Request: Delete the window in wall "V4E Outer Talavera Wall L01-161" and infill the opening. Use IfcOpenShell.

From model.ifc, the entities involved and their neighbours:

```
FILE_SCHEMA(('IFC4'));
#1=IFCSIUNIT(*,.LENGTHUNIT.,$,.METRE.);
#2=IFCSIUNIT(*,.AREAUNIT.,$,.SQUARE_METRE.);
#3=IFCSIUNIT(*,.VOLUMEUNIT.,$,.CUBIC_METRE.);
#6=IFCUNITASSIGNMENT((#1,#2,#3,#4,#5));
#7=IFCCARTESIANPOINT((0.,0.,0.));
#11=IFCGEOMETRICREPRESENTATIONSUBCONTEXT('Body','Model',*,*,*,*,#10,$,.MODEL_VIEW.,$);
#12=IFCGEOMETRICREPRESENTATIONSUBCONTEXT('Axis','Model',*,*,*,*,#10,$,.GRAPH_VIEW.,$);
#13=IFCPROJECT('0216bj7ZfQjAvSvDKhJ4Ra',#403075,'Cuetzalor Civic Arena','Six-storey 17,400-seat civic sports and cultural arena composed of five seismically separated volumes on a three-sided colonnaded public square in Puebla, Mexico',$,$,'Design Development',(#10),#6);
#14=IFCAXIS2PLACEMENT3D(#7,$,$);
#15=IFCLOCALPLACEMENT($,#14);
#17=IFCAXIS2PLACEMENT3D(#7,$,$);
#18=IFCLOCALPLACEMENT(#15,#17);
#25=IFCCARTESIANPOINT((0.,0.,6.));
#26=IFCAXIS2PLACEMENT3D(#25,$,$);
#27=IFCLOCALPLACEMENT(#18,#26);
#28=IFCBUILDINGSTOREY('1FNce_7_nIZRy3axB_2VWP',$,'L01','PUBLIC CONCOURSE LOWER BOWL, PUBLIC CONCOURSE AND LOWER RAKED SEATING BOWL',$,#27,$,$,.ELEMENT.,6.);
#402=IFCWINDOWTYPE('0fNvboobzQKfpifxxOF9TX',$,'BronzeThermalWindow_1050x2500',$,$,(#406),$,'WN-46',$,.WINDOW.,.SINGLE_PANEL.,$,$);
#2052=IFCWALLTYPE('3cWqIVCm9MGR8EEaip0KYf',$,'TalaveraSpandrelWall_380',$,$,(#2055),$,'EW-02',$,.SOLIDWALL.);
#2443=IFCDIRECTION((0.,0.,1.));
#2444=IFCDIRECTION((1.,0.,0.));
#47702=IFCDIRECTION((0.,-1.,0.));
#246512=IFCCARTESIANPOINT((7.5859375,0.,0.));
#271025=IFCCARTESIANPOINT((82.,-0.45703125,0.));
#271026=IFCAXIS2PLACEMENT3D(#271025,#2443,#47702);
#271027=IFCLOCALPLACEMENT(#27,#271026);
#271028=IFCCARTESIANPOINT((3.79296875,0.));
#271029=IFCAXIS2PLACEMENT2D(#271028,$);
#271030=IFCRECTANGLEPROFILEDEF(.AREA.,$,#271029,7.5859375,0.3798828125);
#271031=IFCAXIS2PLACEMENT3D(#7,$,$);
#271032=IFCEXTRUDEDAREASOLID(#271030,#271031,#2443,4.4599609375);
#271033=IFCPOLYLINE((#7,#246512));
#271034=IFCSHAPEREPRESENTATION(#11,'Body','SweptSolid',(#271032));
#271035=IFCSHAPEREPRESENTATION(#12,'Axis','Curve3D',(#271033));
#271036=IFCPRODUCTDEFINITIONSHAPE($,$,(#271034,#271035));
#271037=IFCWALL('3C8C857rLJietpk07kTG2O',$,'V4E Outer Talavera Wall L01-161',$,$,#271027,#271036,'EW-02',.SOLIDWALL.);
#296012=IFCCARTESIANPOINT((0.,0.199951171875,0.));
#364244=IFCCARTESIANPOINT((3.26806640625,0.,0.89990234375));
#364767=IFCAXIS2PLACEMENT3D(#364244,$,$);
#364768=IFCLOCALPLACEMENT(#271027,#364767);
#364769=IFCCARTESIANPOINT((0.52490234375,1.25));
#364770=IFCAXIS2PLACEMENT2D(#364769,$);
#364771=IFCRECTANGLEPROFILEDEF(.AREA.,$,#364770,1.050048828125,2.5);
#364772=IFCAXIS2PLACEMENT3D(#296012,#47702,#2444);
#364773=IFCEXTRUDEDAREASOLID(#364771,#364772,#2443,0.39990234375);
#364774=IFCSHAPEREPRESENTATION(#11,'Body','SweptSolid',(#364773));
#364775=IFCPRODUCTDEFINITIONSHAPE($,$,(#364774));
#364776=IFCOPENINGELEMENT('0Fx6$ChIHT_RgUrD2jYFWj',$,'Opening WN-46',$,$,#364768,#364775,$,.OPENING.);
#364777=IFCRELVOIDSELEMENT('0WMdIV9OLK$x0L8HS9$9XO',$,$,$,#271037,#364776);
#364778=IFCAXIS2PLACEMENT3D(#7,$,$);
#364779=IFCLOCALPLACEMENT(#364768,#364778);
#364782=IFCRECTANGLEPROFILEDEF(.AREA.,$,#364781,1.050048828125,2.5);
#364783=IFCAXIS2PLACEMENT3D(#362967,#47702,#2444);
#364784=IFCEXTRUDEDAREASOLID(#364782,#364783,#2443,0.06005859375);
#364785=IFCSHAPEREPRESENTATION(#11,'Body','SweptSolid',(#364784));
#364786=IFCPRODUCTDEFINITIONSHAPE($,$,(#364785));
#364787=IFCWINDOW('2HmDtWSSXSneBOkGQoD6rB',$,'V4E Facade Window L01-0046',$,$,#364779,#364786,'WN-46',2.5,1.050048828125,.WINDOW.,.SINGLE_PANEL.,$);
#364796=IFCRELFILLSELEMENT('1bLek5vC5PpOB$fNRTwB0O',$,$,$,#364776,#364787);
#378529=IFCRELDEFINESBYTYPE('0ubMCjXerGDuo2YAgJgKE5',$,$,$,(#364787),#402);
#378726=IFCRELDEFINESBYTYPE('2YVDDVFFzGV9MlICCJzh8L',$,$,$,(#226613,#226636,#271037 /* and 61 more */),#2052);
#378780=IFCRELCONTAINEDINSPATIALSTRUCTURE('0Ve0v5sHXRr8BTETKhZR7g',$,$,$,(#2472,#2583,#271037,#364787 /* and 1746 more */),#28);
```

```python
import ifcopenshell
import ifcopenshell.api.feature
import ifcopenshell.api.root
import ifcopenshell.geom
import ifcopenshell.util.shape

model = ifcopenshell.open("model.ifc")
settings = ifcopenshell.geom.settings()


def volume(element):
    """Net volume in cubic metres, openings subtracted."""
    shape = ifcopenshell.geom.create_shape(settings, element)
    return ifcopenshell.util.shape.get_volume(shape.geometry)


window = model.by_guid("2HmDtWSSXSneBOkGQoD6rB")
opening = window.FillsVoids[0].RelatingOpeningElement
wall = opening.VoidsElements[0].RelatingBuildingElement
before = volume(wall)

ifcopenshell.api.root.remove_product(model, product=window)
ifcopenshell.api.feature.remove_feature(model, feature=opening)

after = volume(wall)

print(f"wall volume {before:.3f} -> {after:.3f} m3")

model.write("model_rev.ifc")
```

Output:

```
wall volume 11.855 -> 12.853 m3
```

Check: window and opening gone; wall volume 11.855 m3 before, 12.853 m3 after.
